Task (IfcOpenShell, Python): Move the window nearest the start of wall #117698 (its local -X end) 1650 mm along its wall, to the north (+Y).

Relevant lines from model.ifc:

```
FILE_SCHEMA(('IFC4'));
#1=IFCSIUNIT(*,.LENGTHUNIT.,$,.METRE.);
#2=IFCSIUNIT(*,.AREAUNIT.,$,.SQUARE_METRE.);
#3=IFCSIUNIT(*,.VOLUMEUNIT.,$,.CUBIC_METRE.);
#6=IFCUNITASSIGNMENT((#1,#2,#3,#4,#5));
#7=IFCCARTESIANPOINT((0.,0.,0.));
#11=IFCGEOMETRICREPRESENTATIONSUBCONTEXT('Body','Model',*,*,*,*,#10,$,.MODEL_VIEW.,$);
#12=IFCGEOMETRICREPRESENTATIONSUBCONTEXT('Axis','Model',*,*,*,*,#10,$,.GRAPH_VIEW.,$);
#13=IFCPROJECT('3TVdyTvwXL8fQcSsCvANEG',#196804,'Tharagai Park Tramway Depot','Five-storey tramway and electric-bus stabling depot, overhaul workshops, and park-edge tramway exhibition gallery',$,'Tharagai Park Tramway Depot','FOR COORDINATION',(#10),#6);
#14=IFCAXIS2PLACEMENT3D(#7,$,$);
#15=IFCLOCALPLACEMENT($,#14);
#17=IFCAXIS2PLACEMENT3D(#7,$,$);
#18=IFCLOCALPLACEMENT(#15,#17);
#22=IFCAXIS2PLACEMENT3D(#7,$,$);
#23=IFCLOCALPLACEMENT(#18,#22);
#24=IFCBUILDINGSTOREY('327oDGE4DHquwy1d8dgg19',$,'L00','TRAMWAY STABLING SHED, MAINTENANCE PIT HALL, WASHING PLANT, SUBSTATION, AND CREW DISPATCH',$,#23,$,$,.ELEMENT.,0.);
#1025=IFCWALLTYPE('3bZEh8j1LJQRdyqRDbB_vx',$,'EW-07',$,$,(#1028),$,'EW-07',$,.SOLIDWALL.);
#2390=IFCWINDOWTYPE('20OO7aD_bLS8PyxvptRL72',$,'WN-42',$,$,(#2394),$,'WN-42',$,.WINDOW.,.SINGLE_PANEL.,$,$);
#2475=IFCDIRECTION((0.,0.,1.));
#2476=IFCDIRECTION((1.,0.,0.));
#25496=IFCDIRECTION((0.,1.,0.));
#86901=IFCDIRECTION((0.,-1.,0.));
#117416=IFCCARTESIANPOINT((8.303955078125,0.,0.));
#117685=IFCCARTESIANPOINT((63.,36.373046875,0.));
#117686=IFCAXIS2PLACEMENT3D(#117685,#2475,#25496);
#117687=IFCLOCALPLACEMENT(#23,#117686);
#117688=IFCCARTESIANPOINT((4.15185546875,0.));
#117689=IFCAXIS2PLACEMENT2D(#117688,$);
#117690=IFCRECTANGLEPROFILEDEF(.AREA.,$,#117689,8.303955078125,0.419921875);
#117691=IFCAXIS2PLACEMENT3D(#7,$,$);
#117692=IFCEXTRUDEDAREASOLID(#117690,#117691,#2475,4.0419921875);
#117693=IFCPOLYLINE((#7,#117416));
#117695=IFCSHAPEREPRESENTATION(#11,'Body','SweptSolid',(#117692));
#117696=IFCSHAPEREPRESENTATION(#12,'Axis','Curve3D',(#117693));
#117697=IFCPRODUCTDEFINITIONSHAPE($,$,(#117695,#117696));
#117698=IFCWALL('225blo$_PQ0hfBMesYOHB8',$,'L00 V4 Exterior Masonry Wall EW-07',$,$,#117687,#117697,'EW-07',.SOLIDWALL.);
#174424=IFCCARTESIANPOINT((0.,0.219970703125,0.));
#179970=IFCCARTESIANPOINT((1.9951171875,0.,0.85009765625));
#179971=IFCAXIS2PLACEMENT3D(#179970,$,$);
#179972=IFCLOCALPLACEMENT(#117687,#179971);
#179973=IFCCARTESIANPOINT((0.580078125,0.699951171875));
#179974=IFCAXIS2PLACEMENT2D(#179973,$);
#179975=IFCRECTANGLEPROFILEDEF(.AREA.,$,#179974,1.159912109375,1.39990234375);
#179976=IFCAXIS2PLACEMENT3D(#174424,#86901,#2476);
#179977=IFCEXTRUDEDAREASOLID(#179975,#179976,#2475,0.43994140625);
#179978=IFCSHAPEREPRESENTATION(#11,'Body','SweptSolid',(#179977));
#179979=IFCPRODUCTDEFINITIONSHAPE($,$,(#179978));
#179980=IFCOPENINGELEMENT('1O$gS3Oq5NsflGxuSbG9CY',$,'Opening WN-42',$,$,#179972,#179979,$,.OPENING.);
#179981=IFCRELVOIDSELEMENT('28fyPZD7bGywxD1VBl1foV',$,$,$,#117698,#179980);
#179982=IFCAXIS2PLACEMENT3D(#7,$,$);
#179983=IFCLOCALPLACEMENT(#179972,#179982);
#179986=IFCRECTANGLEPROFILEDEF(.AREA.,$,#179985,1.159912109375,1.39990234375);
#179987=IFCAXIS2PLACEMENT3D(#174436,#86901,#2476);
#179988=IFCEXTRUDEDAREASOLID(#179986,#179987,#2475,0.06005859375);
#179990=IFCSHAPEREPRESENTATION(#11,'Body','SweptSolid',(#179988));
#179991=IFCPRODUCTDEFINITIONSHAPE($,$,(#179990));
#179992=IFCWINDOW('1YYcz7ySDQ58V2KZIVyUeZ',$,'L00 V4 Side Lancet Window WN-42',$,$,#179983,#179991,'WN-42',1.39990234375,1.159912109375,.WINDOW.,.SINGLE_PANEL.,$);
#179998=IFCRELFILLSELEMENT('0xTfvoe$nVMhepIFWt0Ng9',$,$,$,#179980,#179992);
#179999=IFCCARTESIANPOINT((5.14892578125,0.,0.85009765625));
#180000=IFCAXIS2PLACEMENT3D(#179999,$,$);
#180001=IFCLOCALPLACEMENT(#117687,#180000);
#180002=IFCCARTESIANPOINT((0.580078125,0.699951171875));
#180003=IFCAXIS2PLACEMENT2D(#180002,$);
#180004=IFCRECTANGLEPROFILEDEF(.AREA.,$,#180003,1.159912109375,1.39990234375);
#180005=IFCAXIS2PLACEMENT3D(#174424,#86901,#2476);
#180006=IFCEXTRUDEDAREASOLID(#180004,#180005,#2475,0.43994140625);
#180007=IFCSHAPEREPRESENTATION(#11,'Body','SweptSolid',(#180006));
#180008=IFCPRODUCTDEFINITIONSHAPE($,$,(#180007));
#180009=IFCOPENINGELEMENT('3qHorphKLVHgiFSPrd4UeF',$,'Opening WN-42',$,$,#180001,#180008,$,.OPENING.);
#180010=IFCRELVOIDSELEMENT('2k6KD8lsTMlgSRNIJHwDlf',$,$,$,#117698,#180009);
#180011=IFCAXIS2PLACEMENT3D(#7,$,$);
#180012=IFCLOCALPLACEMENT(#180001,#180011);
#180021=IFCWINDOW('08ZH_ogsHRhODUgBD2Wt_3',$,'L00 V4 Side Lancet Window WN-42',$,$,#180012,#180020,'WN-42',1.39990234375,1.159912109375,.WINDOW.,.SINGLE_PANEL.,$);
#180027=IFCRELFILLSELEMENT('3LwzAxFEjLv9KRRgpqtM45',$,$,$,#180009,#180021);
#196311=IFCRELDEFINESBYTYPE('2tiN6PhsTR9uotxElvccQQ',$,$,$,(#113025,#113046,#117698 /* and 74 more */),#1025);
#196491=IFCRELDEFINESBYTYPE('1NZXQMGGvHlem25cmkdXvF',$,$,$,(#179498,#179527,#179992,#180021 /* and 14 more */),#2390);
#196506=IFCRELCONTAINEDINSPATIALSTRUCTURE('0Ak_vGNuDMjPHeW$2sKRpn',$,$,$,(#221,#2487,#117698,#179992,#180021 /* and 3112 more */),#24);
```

```python
import ifcopenshell
import ifcopenshell.api.geometry
import ifcopenshell.util.placement
import ifcopenshell.util.unit

model = ifcopenshell.open("model.ifc")
unit_scale = ifcopenshell.util.unit.calculate_unit_scale(model)

window = model.by_id(179992)
opening = window.FillsVoids[0].RelatingOpeningElement
wall = opening.VoidsElements[0].RelatingBuildingElement

wall_matrix = ifcopenshell.util.placement.get_local_placement(wall.ObjectPlacement)
shift = wall_matrix[:3, 0] * 1.65 / unit_scale
before = ifcopenshell.util.placement.get_local_placement(window.ObjectPlacement)[:3, 3].copy()

# The window is placed relative to its opening, so it follows when the opening moves.
matrix = ifcopenshell.util.placement.get_local_placement(opening.ObjectPlacement)
matrix[:3, 3] += shift
ifcopenshell.api.geometry.edit_object_placement(
    model, product=opening, matrix=matrix, is_si=False, should_transform_children=True
)

after = ifcopenshell.util.placement.get_local_placement(window.ObjectPlacement)[:3, 3]
print("window moved by", (after - before).round(3) + 0.0)

model.write("model_edited.ifc")
```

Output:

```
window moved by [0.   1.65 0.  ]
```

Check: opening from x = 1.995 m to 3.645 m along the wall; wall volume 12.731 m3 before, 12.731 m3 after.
